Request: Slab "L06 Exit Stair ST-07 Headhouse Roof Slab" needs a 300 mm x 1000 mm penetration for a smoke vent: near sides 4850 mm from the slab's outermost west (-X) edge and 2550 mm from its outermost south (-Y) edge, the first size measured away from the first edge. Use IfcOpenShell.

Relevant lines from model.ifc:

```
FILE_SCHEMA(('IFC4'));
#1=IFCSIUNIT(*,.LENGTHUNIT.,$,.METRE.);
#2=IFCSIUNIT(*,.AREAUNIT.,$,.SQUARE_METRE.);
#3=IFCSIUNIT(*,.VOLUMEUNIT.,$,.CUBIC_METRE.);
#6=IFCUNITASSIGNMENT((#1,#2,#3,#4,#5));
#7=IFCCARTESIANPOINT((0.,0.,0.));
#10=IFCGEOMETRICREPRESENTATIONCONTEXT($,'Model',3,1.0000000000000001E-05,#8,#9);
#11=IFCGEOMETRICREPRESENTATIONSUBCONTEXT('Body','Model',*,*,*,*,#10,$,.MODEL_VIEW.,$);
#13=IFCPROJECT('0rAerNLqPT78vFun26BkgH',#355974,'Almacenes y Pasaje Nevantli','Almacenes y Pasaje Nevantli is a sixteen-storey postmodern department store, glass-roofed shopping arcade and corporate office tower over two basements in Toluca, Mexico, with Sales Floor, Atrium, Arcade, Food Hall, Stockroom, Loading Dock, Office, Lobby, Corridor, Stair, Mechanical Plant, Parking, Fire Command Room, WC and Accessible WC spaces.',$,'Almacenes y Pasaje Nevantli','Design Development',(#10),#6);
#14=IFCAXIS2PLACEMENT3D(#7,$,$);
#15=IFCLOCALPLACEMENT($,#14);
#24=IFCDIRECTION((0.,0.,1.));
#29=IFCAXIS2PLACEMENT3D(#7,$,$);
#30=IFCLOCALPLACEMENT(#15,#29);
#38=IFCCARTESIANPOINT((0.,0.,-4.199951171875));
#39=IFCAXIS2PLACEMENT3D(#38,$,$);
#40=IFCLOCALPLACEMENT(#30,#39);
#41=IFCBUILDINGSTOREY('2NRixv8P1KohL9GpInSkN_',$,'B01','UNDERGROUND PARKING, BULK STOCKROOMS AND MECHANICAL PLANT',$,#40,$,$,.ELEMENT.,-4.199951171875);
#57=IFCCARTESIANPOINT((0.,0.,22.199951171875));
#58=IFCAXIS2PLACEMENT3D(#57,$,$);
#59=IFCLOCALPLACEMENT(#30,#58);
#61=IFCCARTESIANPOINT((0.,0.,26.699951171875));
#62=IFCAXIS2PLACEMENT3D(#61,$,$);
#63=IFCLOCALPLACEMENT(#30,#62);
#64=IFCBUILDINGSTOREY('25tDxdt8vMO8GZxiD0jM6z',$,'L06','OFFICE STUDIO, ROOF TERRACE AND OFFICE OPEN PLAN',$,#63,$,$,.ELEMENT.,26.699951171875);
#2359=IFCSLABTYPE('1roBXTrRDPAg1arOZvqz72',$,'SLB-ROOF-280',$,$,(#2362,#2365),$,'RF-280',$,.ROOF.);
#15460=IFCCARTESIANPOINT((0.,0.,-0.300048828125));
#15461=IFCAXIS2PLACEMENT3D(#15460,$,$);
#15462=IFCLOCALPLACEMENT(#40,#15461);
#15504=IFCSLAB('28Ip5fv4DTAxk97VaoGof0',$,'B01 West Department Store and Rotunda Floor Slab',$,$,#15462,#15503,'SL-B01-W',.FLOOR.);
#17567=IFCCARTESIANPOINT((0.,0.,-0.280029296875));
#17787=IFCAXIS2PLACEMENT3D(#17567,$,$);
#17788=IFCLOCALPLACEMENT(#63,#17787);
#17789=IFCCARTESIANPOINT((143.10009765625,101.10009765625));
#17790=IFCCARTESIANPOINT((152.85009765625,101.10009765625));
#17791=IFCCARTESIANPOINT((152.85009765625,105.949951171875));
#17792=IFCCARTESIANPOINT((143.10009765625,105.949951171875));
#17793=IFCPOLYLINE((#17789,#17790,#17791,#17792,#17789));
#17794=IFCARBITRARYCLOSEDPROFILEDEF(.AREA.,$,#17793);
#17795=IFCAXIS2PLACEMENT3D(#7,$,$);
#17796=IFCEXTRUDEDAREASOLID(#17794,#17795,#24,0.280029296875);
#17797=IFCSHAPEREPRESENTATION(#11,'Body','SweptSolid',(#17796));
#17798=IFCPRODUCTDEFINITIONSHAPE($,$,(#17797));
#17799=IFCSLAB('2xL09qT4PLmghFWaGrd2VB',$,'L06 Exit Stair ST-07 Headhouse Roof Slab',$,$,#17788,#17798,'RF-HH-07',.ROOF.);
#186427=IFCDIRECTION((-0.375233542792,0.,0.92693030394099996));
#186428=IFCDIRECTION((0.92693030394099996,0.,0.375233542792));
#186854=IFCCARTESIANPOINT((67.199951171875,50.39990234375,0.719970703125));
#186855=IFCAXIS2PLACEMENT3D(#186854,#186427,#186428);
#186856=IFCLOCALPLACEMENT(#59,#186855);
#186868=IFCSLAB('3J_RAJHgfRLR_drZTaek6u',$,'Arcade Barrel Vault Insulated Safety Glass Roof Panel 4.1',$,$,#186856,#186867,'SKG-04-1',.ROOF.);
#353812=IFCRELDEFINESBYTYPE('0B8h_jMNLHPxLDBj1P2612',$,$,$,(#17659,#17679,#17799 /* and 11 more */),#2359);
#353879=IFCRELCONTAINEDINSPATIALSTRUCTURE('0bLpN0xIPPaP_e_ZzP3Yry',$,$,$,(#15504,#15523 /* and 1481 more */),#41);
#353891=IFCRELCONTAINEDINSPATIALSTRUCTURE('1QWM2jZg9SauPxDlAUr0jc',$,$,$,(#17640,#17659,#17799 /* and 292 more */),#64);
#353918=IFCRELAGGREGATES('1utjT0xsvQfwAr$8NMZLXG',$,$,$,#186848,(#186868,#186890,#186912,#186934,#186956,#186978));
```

```python
import numpy as np
import ifcopenshell
import ifcopenshell.api.feature
import ifcopenshell.api.geometry
import ifcopenshell.api.root
import ifcopenshell.geom
import ifcopenshell.util.placement
import ifcopenshell.util.representation
import ifcopenshell.util.shape
import ifcopenshell.util.unit

model = ifcopenshell.open("model.ifc")
unit_scale = ifcopenshell.util.unit.calculate_unit_scale(model)
settings = ifcopenshell.geom.settings()


def volume(element):
    """Net volume in cubic metres, openings subtracted."""
    shape = ifcopenshell.geom.create_shape(settings, element)
    return ifcopenshell.util.shape.get_volume(shape.geometry)


slab = model.by_guid("2xL09qT4PLmghFWaGrd2VB")
before = volume(slab)

# Extent in the slab's own axes, in metres. The edges named are its -X and -Y sides.
slab_shape = ifcopenshell.geom.create_shape(settings, slab)
vertices = ifcopenshell.util.shape.get_vertices(slab_shape.geometry)
x_min, y_min, bottom = vertices.min(axis=0)
top = vertices[:, 2].max()

opening = ifcopenshell.api.root.create_entity(model, ifc_class="IfcOpeningElement", name="Smoke vent opening", predefined_type="OPENING")
context = ifcopenshell.util.representation.get_context(model, "Model", "Body", "MODEL_VIEW")
width, depth = 0.3, 1
outline = [(0.0, 0.0), (width, 0.0), (width, depth), (0.0, depth), (0.0, 0.0)]
# Overshoot both faces by 50 mm so the cut is clean.
shape = ifcopenshell.api.geometry.add_slab_representation(
    model, context=context, depth=top - bottom + 0.1, polyline=outline
)
ifcopenshell.api.geometry.assign_representation(model, product=opening, representation=shape)

matrix = ifcopenshell.util.placement.get_local_placement(slab.ObjectPlacement)
matrix[:, 3] = matrix @ np.append(np.array([x_min + 4.85, y_min + 2.55, bottom - 0.05]) / unit_scale, 1.0)
ifcopenshell.api.geometry.edit_object_placement(model, product=opening, matrix=matrix, is_si=False)
ifcopenshell.api.feature.add_feature(model, feature=opening, element=slab)

after = volume(slab)

print(f"slab volume {before:.3f} -> {after:.3f} m3")

model.write("model_rev.ifc")
```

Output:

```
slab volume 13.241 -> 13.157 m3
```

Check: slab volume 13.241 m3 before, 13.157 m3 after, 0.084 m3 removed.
